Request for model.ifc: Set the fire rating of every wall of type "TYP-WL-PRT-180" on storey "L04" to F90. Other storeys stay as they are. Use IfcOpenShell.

First a look at what the model holds.

```python
import ifcopenshell
import ifcopenshell.util.element

model = ifcopenshell.open("model.ifc")
print(model.schema)
storey = next(s for s in model.by_type("IfcBuildingStorey") if s.Name == "L04")
walls = [e for e in ifcopenshell.util.element.get_decomposition(storey) if e.is_a("IfcWall")]
seen = {}
for e in walls:
    element_type = ifcopenshell.util.element.get_type(e)
    key = (element_type.Name if element_type != e and element_type else None, ifcopenshell.util.element.get_pset(e, "Pset_WallCommon", "FireRating"))
    seen[key] = seen.get(key, 0) + 1
for (name, value), count in sorted(seen.items(), key=str):
    print(count, "x", name, "|", value)
```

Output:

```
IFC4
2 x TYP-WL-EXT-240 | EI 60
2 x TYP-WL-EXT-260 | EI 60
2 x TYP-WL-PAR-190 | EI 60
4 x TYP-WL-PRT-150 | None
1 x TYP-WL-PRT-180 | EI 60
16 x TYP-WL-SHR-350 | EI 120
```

```python
import ifcopenshell
import ifcopenshell.api.pset
import ifcopenshell.util.element

model = ifcopenshell.open("model.ifc")

storey = next(s for s in model.by_type("IfcBuildingStorey") if s.Name == "L04")
walls = [e for e in ifcopenshell.util.element.get_decomposition(storey) if e.is_a("IfcWall")]

count = 0
for e in walls:
    element_type = ifcopenshell.util.element.get_type(e)
    if element_type in (None, e) or element_type.Name != "TYP-WL-PRT-180":
        continue
    # add_pset returns the element's existing set when there is one.
    pset = ifcopenshell.api.pset.add_pset(model, product=e, name="Pset_WallCommon")
    ifcopenshell.api.pset.edit_pset(model, pset=pset, properties={"FireRating": "F90"})
    count += 1

print(count, "walls updated")

model.write("model_v2.ifc")
```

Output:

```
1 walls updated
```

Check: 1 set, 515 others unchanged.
